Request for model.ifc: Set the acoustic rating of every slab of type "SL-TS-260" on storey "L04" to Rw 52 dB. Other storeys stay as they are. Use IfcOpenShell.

First a look at what the model holds.

```python
import ifcopenshell
import ifcopenshell.util.element

model = ifcopenshell.open("model.ifc")
print(model.schema)
storey = next(s for s in model.by_type("IfcBuildingStorey") if s.Name == "L04")
slabs = [e for e in ifcopenshell.util.element.get_decomposition(storey) if e.is_a("IfcSlab")]
seen = {}
for e in slabs:
    element_type = ifcopenshell.util.element.get_type(e)
    key = (element_type.Name if element_type != e and element_type else None, ifcopenshell.util.element.get_pset(e, "Pset_SlabCommon", "AcousticRating"))
    seen[key] = seen.get(key, 0) + 1
for (name, value), count in sorted(seen.items(), key=str):
    print(count, "x", name, "|", value)
```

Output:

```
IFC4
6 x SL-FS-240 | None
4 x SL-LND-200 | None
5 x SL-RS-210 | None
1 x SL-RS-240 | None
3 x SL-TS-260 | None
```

```python
import ifcopenshell
import ifcopenshell.api.pset
import ifcopenshell.util.element

model = ifcopenshell.open("model.ifc")

storey = next(s for s in model.by_type("IfcBuildingStorey") if s.Name == "L04")
slabs = [e for e in ifcopenshell.util.element.get_decomposition(storey) if e.is_a("IfcSlab")]

count = 0
for e in slabs:
    element_type = ifcopenshell.util.element.get_type(e)
    if element_type in (None, e) or element_type.Name != "SL-TS-260":
        continue
    # add_pset returns the element's existing set when there is one.
    pset = ifcopenshell.api.pset.add_pset(model, product=e, name="Pset_SlabCommon")
    ifcopenshell.api.pset.edit_pset(model, pset=pset, properties={"AcousticRating": "Rw 52 dB"})
    count += 1

print(count, "slabs updated")

model.write("model_v2.ifc")
```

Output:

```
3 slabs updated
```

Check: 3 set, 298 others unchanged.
